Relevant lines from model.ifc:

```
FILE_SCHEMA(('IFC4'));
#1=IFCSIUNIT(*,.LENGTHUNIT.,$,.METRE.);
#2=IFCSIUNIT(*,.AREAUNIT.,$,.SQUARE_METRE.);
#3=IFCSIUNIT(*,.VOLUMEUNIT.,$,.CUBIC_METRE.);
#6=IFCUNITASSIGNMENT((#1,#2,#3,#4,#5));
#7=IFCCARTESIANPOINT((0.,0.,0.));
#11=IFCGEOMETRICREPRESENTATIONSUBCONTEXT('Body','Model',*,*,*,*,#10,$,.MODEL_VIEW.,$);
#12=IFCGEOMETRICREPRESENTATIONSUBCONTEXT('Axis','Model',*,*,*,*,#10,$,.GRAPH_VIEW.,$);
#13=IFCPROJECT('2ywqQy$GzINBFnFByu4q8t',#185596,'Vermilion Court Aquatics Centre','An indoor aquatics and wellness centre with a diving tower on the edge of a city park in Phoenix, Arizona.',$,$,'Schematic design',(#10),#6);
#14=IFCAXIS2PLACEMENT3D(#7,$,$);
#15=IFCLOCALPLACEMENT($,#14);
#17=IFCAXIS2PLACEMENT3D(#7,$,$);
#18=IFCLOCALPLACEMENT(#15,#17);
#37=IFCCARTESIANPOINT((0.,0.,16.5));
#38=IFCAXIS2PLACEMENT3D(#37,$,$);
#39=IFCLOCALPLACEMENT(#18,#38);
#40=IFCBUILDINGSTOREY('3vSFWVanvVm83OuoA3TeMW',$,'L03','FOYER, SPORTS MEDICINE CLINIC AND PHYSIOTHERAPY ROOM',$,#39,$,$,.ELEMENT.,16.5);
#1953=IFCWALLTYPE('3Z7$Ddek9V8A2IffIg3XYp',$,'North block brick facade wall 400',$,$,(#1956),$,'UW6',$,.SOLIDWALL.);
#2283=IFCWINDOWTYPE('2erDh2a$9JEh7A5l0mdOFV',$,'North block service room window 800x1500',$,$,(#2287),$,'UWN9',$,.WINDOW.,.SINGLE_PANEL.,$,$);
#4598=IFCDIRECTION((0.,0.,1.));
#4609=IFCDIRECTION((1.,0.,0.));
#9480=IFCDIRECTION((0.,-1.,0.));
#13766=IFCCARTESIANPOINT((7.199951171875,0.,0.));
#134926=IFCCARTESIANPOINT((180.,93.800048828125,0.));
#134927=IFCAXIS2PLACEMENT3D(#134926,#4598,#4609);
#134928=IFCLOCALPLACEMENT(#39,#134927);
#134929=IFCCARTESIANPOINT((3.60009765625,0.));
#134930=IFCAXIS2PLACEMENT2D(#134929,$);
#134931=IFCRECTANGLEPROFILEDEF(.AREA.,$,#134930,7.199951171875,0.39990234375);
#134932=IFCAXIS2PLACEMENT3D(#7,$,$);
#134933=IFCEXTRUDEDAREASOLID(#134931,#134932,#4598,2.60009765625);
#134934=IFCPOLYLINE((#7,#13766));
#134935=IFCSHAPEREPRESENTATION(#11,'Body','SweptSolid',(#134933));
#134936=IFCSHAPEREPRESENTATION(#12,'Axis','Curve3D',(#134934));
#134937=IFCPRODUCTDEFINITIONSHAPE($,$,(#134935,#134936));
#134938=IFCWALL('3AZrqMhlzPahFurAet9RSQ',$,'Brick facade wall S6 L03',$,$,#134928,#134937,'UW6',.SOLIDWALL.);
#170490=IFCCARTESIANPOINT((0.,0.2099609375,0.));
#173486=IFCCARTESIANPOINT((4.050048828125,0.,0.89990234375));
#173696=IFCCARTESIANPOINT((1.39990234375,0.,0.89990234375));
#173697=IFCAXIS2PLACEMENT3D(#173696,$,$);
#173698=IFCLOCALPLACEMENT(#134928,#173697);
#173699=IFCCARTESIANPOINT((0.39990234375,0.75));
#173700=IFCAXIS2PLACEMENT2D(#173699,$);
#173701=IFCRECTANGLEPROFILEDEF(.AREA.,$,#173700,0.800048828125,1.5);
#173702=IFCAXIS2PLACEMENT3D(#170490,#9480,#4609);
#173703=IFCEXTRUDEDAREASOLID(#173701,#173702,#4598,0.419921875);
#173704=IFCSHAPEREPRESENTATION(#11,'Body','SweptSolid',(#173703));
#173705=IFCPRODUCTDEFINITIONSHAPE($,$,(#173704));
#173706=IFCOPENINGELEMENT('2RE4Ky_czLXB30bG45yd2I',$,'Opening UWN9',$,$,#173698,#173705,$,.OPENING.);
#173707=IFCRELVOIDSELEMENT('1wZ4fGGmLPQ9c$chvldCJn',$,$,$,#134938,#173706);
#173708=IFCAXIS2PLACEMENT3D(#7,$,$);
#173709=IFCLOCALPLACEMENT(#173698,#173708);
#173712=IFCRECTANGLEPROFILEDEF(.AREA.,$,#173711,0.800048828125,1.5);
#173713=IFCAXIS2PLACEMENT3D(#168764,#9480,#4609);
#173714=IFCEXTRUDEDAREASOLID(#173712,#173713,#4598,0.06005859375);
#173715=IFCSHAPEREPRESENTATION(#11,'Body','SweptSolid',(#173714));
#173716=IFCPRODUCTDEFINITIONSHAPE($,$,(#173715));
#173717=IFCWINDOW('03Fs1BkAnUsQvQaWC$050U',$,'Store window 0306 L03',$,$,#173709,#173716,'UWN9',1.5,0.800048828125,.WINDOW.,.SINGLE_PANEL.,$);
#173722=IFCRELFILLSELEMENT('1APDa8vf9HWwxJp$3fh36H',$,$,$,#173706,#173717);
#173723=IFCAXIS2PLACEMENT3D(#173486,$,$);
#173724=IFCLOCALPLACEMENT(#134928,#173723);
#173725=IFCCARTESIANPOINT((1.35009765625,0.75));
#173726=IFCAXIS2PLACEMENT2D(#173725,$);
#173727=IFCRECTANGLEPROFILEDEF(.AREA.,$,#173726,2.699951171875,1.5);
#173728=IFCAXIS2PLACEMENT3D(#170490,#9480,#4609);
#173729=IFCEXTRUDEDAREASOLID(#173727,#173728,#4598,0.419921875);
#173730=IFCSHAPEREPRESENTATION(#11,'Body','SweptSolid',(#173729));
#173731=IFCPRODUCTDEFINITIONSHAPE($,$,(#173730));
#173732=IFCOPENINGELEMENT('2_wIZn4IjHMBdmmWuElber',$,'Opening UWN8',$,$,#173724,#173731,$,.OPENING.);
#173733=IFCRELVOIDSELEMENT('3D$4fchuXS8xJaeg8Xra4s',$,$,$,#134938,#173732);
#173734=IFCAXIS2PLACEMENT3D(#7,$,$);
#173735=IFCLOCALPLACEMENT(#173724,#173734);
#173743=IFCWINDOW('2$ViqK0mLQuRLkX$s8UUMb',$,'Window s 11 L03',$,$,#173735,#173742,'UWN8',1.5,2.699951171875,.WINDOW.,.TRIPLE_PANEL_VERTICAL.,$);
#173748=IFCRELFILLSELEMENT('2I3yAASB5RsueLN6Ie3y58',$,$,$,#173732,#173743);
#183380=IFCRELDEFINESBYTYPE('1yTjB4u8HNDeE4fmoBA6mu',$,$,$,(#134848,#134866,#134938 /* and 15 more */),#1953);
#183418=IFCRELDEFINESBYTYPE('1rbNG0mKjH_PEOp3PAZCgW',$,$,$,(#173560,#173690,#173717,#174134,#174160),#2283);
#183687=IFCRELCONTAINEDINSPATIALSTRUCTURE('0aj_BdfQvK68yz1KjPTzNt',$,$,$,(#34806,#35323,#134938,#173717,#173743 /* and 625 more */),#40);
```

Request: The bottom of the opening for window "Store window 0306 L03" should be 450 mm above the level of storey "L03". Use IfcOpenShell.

```python
import numpy as np
import ifcopenshell
import ifcopenshell.api.geometry
import ifcopenshell.geom
import ifcopenshell.util.element
import ifcopenshell.util.placement
import ifcopenshell.util.shape
import ifcopenshell.util.unit

model = ifcopenshell.open("model.ifc")
unit_scale = ifcopenshell.util.unit.calculate_unit_scale(model)

window = model.by_id(173717)
opening = window.FillsVoids[0].RelatingOpeningElement
storey = ifcopenshell.util.element.get_container(window, ifc_class="IfcBuildingStorey")
level = ifcopenshell.util.placement.get_local_placement(storey.ObjectPlacement)[2, 3]

# The opening's origin need not be at the sill, so measure its lowest point.
shape = ifcopenshell.geom.create_shape(ifcopenshell.geom.settings(), opening)
bottom = ifcopenshell.util.shape.get_shape_bottom_elevation(shape, shape.geometry) / unit_scale
dz = level + 0.45 / unit_scale - bottom

shift = np.array([0.0, 0.0, dz])
# The window is placed relative to its opening, so it follows when the opening moves.
matrix = ifcopenshell.util.placement.get_local_placement(opening.ObjectPlacement)
matrix[:3, 3] += shift
ifcopenshell.api.geometry.edit_object_placement(
    model, product=opening, matrix=matrix, is_si=False, should_transform_children=True
)

print(f"moved by {dz * unit_scale:+.3f} m")

model.write("model_rev.ifc")
```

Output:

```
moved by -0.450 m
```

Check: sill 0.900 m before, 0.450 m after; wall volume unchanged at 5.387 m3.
